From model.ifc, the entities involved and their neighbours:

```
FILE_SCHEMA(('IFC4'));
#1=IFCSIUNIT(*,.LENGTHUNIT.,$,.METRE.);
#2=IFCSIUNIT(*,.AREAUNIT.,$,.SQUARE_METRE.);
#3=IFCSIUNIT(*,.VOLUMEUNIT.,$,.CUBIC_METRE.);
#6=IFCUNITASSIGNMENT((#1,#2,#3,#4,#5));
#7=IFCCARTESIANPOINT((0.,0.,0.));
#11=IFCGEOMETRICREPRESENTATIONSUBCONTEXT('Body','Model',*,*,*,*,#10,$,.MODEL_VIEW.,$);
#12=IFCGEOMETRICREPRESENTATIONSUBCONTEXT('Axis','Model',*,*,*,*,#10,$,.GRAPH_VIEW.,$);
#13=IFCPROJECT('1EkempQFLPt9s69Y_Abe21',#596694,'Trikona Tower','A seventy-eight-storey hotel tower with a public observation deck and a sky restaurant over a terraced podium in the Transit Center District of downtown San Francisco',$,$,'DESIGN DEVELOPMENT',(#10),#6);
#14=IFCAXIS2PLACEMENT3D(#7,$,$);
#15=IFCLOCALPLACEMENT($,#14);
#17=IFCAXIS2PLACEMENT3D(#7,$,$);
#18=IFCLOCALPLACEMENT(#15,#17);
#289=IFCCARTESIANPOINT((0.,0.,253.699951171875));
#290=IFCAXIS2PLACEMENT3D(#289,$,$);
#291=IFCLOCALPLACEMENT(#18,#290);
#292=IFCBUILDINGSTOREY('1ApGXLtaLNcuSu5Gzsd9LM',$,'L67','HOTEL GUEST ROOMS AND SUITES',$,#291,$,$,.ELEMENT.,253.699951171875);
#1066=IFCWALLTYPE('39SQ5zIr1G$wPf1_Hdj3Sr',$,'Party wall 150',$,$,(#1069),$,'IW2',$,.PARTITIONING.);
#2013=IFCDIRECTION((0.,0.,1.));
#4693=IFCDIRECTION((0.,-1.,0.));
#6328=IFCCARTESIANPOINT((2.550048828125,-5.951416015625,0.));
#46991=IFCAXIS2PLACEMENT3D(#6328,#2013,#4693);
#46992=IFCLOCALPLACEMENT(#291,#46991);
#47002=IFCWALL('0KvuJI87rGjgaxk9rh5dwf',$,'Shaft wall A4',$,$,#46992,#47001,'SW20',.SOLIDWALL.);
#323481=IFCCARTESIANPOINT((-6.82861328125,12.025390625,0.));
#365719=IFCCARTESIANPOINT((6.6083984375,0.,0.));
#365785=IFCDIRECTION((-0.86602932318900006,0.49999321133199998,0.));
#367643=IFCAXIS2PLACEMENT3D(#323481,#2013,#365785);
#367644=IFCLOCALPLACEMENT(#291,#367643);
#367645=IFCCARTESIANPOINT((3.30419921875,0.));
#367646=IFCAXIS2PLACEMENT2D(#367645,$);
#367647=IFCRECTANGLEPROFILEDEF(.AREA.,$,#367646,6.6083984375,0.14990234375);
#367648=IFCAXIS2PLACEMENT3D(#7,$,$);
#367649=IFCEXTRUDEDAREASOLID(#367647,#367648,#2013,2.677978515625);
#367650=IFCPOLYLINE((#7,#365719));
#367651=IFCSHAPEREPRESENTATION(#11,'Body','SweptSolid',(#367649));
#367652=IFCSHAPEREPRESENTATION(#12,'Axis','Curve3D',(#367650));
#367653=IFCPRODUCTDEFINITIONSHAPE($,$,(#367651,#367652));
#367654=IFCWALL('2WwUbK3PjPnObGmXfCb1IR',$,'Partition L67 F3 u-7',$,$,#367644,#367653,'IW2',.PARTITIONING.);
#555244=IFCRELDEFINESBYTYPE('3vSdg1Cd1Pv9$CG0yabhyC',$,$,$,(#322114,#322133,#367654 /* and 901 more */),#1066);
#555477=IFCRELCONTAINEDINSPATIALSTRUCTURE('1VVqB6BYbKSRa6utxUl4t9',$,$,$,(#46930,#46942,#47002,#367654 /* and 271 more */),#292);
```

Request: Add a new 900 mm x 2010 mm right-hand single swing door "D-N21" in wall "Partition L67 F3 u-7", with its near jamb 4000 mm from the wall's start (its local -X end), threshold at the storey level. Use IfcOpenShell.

```python
import numpy as np
import ifcopenshell
import ifcopenshell.api.feature
import ifcopenshell.api.geometry
import ifcopenshell.api.root
import ifcopenshell.api.spatial
import ifcopenshell.geom
import ifcopenshell.util.element
import ifcopenshell.util.placement
import ifcopenshell.util.representation
import ifcopenshell.util.shape
import ifcopenshell.util.unit

model = ifcopenshell.open("model.ifc")
unit_scale = ifcopenshell.util.unit.calculate_unit_scale(model)
settings = ifcopenshell.geom.settings()


def volume(element):
    """Net volume in cubic metres, openings subtracted."""
    shape = ifcopenshell.geom.create_shape(settings, element)
    return ifcopenshell.util.shape.get_volume(shape.geometry)


wall = model.by_guid("2WwUbK3PjPnObGmXfCb1IR")
storey = ifcopenshell.util.element.get_container(wall, ifc_class="IfcBuildingStorey")
context = ifcopenshell.util.representation.get_context(model, "Model", "Body", "MODEL_VIEW")
before = volume(wall)

width, height, from_end, sill = 0.9, 2.01, 4, 0.0  # metres

# The wall runs along its own X axis, and the end named is its -X end.
wall_shape = ifcopenshell.geom.create_shape(settings, wall)
x, y, z = ifcopenshell.util.shape.get_vertices(wall_shape.geometry).T
start = x.min() + from_end
face, thickness = float(y.min()), float(y.max() - y.min())
wall_matrix = ifcopenshell.util.placement.get_local_placement(wall.ObjectPlacement)
level = ifcopenshell.util.placement.get_local_placement(storey.ObjectPlacement)[2, 3]


def in_wall(x, y):
    """Placement at x, y metres in the wall's axes, at sill height."""
    matrix = wall_matrix.copy()
    matrix[:, 3] = wall_matrix @ np.array([x / unit_scale, y / unit_scale, 0.0, 1.0])
    matrix[2, 3] = level + sill / unit_scale
    return matrix


# Opening: a box that overshoots both wall faces by 50 mm.
opening = ifcopenshell.api.root.create_entity(model, ifc_class="IfcOpeningElement", predefined_type="OPENING")
box = ifcopenshell.api.geometry.add_wall_representation(
    model, context=context, length=width, height=height, thickness=thickness + 0.1
)
ifcopenshell.api.geometry.assign_representation(model, product=opening, representation=box)
ifcopenshell.api.geometry.edit_object_placement(model, product=opening, matrix=in_wall(start, face - 0.05), is_si=False)
ifcopenshell.api.feature.add_feature(model, feature=opening, element=wall)

door = ifcopenshell.api.root.create_entity(model, ifc_class="IfcDoor", name="D-N21", predefined_type="DOOR")
door.OverallWidth, door.OverallHeight = width / unit_scale, height / unit_scale
door.OperationType = "SINGLE_SWING_RIGHT"
body = ifcopenshell.api.geometry.add_door_representation(
    model,
    context=context,
    overall_width=door.OverallWidth,
    overall_height=door.OverallHeight,
    operation_type="SINGLE_SWING_RIGHT",
    lining_properties={"LiningDepth": thickness / unit_scale, "ThresholdDepth": thickness / unit_scale},
)
ifcopenshell.api.geometry.assign_representation(model, product=door, representation=body)
ifcopenshell.api.spatial.assign_container(model, products=[door], relating_structure=storey)
ifcopenshell.api.feature.add_filling(model, opening=opening, element=door)

# The lining spans the wall, so the door starts at the wall face.
ifcopenshell.api.geometry.edit_object_placement(model, product=door, matrix=in_wall(start, face), is_si=False)

after = volume(wall)

print(f"wall volume {before:.3f} -> {after:.3f} m3")

model.write("model_v2.ifc")
```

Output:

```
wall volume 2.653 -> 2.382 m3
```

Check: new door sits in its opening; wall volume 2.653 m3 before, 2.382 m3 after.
